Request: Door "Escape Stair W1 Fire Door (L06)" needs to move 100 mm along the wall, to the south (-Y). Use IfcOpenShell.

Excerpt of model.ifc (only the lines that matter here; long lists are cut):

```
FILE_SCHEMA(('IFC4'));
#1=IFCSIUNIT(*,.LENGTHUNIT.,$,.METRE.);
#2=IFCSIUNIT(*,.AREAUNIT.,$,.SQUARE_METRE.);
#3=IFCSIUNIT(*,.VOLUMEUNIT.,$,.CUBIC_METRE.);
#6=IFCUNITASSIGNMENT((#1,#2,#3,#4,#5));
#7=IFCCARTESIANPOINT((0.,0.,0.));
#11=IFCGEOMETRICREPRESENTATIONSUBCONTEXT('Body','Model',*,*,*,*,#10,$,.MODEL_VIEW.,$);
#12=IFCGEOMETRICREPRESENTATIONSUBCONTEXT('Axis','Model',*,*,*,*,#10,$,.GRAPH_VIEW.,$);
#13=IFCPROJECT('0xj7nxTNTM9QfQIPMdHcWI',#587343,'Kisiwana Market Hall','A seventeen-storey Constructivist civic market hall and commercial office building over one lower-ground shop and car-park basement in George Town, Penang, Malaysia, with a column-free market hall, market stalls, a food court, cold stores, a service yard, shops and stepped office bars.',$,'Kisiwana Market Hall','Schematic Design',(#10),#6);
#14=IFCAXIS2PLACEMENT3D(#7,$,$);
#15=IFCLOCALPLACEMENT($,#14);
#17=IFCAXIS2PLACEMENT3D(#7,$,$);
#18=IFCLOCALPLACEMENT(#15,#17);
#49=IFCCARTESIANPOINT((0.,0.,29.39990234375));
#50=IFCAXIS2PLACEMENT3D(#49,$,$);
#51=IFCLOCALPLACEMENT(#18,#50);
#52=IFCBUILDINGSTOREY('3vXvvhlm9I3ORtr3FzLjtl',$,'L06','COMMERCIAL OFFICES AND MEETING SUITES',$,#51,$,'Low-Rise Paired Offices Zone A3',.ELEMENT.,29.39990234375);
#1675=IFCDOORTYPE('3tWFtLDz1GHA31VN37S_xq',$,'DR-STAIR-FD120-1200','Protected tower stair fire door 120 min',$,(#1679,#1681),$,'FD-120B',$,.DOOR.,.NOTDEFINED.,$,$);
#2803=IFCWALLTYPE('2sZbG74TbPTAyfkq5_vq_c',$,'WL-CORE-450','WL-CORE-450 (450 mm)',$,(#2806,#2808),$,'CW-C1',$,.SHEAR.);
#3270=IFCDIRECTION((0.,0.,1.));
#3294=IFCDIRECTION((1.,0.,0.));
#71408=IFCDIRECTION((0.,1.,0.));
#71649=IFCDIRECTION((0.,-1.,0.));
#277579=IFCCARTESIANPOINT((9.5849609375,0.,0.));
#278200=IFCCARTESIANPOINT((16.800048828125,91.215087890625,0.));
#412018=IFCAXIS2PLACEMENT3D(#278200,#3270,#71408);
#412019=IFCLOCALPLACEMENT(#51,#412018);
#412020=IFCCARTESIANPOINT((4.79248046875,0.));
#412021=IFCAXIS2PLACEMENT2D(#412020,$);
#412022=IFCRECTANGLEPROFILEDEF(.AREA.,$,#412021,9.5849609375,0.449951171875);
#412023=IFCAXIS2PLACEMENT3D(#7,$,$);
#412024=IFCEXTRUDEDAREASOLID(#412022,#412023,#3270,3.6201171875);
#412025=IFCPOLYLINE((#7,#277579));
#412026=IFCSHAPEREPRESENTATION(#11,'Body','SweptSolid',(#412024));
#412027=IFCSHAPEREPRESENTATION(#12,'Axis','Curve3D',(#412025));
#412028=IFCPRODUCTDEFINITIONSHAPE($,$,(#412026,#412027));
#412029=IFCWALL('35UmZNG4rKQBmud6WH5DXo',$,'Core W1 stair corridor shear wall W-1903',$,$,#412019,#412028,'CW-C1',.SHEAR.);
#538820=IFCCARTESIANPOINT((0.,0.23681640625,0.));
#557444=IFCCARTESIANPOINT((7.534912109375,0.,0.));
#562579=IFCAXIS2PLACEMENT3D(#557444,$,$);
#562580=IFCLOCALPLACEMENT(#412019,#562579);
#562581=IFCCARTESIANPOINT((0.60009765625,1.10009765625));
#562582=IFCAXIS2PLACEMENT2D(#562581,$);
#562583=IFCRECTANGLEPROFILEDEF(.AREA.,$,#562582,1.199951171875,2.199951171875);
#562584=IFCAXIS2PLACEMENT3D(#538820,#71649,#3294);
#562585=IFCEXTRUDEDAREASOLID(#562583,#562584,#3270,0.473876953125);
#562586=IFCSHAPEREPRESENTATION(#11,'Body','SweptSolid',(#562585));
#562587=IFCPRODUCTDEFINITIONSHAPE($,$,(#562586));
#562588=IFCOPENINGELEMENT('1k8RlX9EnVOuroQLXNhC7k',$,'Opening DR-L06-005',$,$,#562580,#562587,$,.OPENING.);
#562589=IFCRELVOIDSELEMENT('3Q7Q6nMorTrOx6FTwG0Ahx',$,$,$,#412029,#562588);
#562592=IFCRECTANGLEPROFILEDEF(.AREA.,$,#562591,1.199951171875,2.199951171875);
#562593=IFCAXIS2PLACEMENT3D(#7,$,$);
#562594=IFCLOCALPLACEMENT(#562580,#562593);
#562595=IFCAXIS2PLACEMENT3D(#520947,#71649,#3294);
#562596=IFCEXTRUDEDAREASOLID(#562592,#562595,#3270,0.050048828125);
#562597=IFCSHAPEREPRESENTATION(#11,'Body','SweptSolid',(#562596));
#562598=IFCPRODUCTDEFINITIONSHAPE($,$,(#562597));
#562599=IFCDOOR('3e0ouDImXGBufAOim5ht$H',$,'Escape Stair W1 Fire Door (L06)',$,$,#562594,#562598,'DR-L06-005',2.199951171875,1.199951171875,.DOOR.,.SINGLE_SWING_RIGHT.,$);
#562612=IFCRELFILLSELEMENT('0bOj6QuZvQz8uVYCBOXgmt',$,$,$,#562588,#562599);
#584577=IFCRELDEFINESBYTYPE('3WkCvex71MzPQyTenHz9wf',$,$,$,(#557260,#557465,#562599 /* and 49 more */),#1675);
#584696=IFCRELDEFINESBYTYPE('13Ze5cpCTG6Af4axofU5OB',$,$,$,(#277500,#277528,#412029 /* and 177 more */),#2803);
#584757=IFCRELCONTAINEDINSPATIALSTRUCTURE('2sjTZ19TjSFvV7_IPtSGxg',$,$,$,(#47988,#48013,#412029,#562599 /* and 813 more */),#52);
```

```python
import ifcopenshell
import ifcopenshell.api.geometry
import ifcopenshell.util.placement
import ifcopenshell.util.unit

model = ifcopenshell.open("model.ifc")
unit_scale = ifcopenshell.util.unit.calculate_unit_scale(model)

door = model.by_guid("3e0ouDImXGBufAOim5ht$H")
opening = door.FillsVoids[0].RelatingOpeningElement
wall = opening.VoidsElements[0].RelatingBuildingElement

wall_matrix = ifcopenshell.util.placement.get_local_placement(wall.ObjectPlacement)
shift = wall_matrix[:3, 0] * -0.1 / unit_scale
before = ifcopenshell.util.placement.get_local_placement(door.ObjectPlacement)[:3, 3].copy()

# The door is placed relative to its opening, so it follows when the opening moves.
matrix = ifcopenshell.util.placement.get_local_placement(opening.ObjectPlacement)
matrix[:3, 3] += shift
ifcopenshell.api.geometry.edit_object_placement(
    model, product=opening, matrix=matrix, is_si=False, should_transform_children=True
)

after = ifcopenshell.util.placement.get_local_placement(door.ObjectPlacement)[:3, 3]
print("door moved by", (after - before).round(3) + 0.0)

model.write("model_rev.ifc")
```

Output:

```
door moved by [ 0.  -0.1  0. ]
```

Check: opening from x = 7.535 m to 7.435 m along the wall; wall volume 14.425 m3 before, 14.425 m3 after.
